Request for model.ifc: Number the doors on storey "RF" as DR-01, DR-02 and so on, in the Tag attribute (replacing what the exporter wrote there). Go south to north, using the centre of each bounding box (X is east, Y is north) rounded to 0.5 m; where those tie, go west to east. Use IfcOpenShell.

First a look at what the model holds.

```python
import ifcopenshell
import ifcopenshell.util.element
import ifcopenshell.util.placement

model = ifcopenshell.open("model.ifc")
print(model.schema)
storey = next(s for s in model.by_type("IfcBuildingStorey") if s.Name == "RF")
doors = [e for e in ifcopenshell.util.element.get_decomposition(storey) if e.is_a("IfcDoor")]
for e in sorted(doors, key=lambda e: e.id()):
    origin = ifcopenshell.util.placement.get_local_placement(e.ObjectPlacement)[:3, 3]
    print(e.id(), e.Tag, e.Name, origin.round(2) + 0.0, sep=" | ")
```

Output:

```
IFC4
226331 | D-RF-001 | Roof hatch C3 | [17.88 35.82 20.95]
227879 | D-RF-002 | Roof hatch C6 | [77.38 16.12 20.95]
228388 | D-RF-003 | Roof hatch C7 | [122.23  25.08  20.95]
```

```python
import ifcopenshell
import ifcopenshell.geom
import ifcopenshell.util.element
import ifcopenshell.util.shape

model = ifcopenshell.open("model.ifc")
settings = ifcopenshell.geom.settings()
settings.set("use-world-coords", True)


def centre(element):
    shape = ifcopenshell.geom.create_shape(settings, element)
    return ifcopenshell.util.shape.get_bbox_centroid(shape.geometry)


storey = next(s for s in model.by_type("IfcBuildingStorey") if s.Name == "RF")
doors = [e for e in ifcopenshell.util.element.get_decomposition(storey) if e.is_a("IfcDoor")]

# Insertion points can sit at a corner or the storey origin, so sort by the geometry (in metres).
centres = {e: centre(e) for e in doors}
doors.sort(key=lambda e: (round(centres[e][1] / 0.5), centres[e][0]))

for i, e in enumerate(doors, start=1):
    number = f"DR-{i:02d}"
    e.Tag = number
    print(e.id(), number)

model.write("model_rev.ifc")
```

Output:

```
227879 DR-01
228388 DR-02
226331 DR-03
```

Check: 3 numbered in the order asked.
